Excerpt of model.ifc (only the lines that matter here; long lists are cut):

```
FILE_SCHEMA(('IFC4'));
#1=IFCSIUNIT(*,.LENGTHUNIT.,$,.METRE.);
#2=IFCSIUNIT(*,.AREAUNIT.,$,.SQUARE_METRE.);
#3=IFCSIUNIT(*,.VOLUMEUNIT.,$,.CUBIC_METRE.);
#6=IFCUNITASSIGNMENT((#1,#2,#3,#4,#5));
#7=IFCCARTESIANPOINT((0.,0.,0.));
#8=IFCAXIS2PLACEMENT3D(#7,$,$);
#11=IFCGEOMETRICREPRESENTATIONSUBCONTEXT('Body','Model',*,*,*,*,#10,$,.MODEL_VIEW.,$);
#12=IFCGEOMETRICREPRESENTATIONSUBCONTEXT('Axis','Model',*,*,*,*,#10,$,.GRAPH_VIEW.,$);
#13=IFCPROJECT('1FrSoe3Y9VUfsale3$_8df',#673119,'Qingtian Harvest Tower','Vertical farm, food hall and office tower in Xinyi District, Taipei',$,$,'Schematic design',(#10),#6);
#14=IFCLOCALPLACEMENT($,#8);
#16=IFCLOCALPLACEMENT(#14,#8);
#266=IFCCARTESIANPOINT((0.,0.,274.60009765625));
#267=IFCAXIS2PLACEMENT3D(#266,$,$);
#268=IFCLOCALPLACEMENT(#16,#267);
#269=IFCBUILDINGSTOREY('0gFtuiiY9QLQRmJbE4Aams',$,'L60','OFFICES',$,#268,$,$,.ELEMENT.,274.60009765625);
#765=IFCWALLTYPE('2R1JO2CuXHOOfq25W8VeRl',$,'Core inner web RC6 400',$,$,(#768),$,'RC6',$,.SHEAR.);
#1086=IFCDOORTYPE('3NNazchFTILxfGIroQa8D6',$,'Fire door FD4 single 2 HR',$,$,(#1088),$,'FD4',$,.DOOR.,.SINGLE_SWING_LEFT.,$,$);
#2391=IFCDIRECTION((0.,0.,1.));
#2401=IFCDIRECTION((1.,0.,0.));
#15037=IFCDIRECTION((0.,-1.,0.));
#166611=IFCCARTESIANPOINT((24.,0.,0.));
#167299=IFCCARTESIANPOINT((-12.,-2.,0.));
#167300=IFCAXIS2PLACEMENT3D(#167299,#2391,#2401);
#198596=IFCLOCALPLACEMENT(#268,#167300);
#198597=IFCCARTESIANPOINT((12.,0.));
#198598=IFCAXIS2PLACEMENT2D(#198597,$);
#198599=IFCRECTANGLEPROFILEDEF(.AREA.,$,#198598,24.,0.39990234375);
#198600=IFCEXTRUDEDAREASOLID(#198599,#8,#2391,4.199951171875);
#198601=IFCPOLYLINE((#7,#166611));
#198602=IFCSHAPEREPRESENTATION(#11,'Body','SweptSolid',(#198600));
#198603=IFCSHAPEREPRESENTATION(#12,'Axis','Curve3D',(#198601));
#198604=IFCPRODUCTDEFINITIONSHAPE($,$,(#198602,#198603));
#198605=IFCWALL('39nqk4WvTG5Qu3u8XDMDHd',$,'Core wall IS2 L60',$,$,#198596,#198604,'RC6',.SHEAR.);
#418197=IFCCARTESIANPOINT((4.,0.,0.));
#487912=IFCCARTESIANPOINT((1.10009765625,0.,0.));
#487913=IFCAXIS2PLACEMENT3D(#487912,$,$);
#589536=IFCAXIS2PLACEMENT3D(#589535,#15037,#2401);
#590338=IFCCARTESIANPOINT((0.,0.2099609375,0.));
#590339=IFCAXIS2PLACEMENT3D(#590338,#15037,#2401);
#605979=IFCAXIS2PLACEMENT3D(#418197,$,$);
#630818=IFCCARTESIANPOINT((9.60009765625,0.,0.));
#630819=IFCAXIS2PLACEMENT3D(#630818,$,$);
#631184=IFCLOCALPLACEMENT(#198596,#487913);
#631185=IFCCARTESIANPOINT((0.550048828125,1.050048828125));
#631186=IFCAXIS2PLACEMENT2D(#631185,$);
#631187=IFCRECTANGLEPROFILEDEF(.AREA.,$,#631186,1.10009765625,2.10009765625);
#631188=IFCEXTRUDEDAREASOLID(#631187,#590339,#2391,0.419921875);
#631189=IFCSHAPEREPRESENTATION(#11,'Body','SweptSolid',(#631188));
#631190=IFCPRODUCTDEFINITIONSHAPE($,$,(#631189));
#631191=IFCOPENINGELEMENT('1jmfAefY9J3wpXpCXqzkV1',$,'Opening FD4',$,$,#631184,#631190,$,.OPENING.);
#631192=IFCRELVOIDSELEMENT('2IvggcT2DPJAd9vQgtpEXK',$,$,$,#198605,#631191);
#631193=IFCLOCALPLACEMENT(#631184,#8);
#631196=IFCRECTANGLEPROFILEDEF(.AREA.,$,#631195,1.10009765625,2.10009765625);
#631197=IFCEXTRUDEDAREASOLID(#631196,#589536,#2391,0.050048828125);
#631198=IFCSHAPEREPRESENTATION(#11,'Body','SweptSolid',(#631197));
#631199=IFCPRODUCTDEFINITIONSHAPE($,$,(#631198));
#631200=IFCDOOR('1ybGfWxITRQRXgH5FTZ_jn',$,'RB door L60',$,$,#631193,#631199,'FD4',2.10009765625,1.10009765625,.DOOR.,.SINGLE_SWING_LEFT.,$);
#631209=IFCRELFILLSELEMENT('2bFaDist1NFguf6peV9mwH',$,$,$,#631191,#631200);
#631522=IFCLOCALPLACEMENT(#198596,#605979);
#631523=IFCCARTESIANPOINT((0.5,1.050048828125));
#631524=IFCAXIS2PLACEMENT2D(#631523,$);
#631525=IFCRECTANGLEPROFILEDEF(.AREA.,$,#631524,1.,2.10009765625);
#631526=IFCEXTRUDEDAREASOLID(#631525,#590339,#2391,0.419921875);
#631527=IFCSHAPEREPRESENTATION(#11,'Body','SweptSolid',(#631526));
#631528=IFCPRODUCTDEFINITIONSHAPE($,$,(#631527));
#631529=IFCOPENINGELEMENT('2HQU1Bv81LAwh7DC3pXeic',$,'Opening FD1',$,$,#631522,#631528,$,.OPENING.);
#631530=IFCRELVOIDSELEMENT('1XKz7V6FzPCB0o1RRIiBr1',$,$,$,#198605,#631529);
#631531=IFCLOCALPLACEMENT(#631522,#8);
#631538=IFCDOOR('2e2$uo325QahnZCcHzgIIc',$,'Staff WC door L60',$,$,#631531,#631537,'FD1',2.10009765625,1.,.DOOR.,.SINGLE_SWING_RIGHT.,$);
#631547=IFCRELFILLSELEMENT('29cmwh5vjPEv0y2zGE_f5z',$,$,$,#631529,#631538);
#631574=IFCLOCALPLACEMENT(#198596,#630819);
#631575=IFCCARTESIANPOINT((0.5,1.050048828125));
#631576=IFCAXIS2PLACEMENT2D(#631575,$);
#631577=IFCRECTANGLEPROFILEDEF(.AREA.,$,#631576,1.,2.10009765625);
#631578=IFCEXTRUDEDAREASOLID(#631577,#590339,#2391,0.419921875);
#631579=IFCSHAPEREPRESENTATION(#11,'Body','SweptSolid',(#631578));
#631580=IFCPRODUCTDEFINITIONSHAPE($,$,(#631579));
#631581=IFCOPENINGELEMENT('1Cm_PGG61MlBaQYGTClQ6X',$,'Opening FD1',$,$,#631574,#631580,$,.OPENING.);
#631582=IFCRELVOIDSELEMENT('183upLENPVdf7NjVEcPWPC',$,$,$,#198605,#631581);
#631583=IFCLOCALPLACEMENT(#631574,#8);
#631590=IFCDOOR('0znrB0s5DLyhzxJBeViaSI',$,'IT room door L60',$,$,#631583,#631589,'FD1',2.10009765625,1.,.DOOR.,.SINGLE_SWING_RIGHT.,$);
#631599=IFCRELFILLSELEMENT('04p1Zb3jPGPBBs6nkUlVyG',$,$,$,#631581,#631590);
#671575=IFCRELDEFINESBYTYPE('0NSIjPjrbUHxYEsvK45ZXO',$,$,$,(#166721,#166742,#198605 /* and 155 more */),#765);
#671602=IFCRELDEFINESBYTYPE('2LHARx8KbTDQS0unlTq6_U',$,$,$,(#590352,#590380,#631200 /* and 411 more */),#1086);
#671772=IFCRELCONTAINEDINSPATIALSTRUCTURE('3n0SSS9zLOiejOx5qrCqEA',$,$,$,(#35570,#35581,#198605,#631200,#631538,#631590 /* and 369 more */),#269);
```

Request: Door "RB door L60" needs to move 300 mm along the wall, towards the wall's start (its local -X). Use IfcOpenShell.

```python
import ifcopenshell
import ifcopenshell.api.geometry
import ifcopenshell.util.placement

model = ifcopenshell.open("model.ifc")

door = model.by_guid("1ybGfWxITRQRXgH5FTZ_jn")
opening = door.FillsVoids[0].RelatingOpeningElement
wall = opening.VoidsElements[0].RelatingBuildingElement

wall_matrix = ifcopenshell.util.placement.get_local_placement(wall.ObjectPlacement)
shift = wall_matrix[:3, 0] * -0.3
before = ifcopenshell.util.placement.get_local_placement(door.ObjectPlacement)[:3, 3].copy()

# The door is placed relative to its opening, so it follows when the opening moves.
matrix = ifcopenshell.util.placement.get_local_placement(opening.ObjectPlacement)
matrix[:3, 3] += shift
ifcopenshell.api.geometry.edit_object_placement(
    model, product=opening, matrix=matrix, is_si=False, should_transform_children=True
)

after = ifcopenshell.util.placement.get_local_placement(door.ObjectPlacement)[:3, 3]
print("door moved by", (after - before).round(3) + 0.0)

model.write("model_edited.ifc")
```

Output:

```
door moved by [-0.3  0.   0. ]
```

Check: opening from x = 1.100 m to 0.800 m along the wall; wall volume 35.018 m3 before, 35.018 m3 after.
